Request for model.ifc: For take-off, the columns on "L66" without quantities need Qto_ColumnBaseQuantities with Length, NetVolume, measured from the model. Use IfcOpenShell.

First a look at what the model holds.

```python
import ifcopenshell
import ifcopenshell.util.element
import ifcopenshell.util.unit

model = ifcopenshell.open("model.ifc")
print(model.schema)
for unit_type in ("LENGTHUNIT", "AREAUNIT", "VOLUMEUNIT"):
    print(unit_type, ifcopenshell.util.unit.calculate_unit_scale(model, unit_type))
storey = next(s for s in model.by_type("IfcBuildingStorey") if s.Name == "L66")
columns = [e for e in ifcopenshell.util.element.get_decomposition(storey) if e.is_a("IfcColumn")]
for e in sorted(columns, key=lambda e: e.id()):
    print(e.id(), e.is_a(), e.Name, list(ifcopenshell.util.element.get_psets(e, qtos_only=True)), sep=" | ")
```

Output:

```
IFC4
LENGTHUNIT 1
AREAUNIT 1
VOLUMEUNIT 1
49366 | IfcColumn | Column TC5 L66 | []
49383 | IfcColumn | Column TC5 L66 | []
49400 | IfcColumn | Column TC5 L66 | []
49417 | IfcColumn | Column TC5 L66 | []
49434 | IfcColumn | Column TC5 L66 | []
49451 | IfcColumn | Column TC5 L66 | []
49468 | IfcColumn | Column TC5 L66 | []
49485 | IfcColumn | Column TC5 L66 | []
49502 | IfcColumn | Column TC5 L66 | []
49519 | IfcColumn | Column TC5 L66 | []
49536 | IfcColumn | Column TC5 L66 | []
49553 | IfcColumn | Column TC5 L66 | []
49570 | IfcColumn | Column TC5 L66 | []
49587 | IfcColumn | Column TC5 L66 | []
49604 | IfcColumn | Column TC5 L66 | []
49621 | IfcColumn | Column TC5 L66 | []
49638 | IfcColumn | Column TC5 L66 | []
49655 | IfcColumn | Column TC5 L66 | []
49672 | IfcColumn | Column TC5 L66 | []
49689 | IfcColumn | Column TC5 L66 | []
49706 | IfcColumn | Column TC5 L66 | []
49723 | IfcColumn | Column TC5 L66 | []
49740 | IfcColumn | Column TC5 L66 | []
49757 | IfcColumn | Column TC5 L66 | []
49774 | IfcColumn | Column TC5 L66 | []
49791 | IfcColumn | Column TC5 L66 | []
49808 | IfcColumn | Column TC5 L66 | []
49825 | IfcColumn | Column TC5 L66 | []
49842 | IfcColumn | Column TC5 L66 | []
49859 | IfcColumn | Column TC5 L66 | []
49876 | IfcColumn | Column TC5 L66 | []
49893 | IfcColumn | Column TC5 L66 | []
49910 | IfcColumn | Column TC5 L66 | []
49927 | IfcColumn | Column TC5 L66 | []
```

```python
import ifcopenshell
import ifcopenshell.api.pset
import ifcopenshell.geom
import ifcopenshell.util.element
import ifcopenshell.util.shape
import ifcopenshell.util.unit

model = ifcopenshell.open("model.ifc")
unit_scale = ifcopenshell.util.unit.calculate_unit_scale(model)
volume_scale = ifcopenshell.util.unit.calculate_unit_scale(model, "VOLUMEUNIT")
settings = ifcopenshell.geom.settings()

storey = next(s for s in model.by_type("IfcBuildingStorey") if s.Name == "L66")
columns = [e for e in ifcopenshell.util.element.get_decomposition(storey) if e.is_a("IfcColumn")]

for e in sorted(columns, key=lambda e: e.id()):
    if ifcopenshell.util.element.get_psets(e, qtos_only=True, should_inherit=False):
        continue
    # Geometry comes back in metres, in the element's own axes.
    shape = ifcopenshell.geom.create_shape(settings, e)
    values = {
        "Length": ifcopenshell.util.shape.get_z(shape.geometry) / unit_scale,
        "NetVolume": ifcopenshell.util.shape.get_volume(shape.geometry) / volume_scale,
    }
    qto = ifcopenshell.api.pset.add_qto(model, product=e, name="Qto_ColumnBaseQuantities")
    ifcopenshell.api.pset.edit_qto(model, qto=qto, properties=values)
    print(e.id(), {k: round(v, 3) for k, v in values.items()})

model.write("model_rev.ifc")
```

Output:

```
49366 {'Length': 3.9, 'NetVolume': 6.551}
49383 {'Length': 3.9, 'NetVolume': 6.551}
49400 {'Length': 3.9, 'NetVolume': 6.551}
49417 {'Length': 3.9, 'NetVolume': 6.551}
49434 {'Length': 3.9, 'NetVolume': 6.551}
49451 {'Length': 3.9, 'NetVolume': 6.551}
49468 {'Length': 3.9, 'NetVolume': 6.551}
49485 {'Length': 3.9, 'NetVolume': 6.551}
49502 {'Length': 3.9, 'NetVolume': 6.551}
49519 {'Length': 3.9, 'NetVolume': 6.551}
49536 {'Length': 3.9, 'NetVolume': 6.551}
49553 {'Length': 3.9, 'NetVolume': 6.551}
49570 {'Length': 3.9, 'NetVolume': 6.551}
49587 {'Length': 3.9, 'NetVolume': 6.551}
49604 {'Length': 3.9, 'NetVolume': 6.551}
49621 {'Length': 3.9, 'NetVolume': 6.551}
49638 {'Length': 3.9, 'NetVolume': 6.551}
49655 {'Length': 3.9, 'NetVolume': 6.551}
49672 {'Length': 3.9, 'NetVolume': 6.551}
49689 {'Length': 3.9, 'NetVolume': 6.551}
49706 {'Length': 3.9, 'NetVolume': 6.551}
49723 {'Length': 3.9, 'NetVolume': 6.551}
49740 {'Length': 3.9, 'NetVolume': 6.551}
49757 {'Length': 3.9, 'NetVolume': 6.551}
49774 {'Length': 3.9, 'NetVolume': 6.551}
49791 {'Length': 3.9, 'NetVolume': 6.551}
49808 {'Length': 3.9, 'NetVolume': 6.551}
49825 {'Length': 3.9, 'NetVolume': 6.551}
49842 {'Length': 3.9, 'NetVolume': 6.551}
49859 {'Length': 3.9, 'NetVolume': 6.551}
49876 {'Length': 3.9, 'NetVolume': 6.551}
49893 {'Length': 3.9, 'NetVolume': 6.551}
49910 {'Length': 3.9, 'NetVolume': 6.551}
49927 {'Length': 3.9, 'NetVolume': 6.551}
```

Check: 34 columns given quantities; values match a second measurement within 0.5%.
